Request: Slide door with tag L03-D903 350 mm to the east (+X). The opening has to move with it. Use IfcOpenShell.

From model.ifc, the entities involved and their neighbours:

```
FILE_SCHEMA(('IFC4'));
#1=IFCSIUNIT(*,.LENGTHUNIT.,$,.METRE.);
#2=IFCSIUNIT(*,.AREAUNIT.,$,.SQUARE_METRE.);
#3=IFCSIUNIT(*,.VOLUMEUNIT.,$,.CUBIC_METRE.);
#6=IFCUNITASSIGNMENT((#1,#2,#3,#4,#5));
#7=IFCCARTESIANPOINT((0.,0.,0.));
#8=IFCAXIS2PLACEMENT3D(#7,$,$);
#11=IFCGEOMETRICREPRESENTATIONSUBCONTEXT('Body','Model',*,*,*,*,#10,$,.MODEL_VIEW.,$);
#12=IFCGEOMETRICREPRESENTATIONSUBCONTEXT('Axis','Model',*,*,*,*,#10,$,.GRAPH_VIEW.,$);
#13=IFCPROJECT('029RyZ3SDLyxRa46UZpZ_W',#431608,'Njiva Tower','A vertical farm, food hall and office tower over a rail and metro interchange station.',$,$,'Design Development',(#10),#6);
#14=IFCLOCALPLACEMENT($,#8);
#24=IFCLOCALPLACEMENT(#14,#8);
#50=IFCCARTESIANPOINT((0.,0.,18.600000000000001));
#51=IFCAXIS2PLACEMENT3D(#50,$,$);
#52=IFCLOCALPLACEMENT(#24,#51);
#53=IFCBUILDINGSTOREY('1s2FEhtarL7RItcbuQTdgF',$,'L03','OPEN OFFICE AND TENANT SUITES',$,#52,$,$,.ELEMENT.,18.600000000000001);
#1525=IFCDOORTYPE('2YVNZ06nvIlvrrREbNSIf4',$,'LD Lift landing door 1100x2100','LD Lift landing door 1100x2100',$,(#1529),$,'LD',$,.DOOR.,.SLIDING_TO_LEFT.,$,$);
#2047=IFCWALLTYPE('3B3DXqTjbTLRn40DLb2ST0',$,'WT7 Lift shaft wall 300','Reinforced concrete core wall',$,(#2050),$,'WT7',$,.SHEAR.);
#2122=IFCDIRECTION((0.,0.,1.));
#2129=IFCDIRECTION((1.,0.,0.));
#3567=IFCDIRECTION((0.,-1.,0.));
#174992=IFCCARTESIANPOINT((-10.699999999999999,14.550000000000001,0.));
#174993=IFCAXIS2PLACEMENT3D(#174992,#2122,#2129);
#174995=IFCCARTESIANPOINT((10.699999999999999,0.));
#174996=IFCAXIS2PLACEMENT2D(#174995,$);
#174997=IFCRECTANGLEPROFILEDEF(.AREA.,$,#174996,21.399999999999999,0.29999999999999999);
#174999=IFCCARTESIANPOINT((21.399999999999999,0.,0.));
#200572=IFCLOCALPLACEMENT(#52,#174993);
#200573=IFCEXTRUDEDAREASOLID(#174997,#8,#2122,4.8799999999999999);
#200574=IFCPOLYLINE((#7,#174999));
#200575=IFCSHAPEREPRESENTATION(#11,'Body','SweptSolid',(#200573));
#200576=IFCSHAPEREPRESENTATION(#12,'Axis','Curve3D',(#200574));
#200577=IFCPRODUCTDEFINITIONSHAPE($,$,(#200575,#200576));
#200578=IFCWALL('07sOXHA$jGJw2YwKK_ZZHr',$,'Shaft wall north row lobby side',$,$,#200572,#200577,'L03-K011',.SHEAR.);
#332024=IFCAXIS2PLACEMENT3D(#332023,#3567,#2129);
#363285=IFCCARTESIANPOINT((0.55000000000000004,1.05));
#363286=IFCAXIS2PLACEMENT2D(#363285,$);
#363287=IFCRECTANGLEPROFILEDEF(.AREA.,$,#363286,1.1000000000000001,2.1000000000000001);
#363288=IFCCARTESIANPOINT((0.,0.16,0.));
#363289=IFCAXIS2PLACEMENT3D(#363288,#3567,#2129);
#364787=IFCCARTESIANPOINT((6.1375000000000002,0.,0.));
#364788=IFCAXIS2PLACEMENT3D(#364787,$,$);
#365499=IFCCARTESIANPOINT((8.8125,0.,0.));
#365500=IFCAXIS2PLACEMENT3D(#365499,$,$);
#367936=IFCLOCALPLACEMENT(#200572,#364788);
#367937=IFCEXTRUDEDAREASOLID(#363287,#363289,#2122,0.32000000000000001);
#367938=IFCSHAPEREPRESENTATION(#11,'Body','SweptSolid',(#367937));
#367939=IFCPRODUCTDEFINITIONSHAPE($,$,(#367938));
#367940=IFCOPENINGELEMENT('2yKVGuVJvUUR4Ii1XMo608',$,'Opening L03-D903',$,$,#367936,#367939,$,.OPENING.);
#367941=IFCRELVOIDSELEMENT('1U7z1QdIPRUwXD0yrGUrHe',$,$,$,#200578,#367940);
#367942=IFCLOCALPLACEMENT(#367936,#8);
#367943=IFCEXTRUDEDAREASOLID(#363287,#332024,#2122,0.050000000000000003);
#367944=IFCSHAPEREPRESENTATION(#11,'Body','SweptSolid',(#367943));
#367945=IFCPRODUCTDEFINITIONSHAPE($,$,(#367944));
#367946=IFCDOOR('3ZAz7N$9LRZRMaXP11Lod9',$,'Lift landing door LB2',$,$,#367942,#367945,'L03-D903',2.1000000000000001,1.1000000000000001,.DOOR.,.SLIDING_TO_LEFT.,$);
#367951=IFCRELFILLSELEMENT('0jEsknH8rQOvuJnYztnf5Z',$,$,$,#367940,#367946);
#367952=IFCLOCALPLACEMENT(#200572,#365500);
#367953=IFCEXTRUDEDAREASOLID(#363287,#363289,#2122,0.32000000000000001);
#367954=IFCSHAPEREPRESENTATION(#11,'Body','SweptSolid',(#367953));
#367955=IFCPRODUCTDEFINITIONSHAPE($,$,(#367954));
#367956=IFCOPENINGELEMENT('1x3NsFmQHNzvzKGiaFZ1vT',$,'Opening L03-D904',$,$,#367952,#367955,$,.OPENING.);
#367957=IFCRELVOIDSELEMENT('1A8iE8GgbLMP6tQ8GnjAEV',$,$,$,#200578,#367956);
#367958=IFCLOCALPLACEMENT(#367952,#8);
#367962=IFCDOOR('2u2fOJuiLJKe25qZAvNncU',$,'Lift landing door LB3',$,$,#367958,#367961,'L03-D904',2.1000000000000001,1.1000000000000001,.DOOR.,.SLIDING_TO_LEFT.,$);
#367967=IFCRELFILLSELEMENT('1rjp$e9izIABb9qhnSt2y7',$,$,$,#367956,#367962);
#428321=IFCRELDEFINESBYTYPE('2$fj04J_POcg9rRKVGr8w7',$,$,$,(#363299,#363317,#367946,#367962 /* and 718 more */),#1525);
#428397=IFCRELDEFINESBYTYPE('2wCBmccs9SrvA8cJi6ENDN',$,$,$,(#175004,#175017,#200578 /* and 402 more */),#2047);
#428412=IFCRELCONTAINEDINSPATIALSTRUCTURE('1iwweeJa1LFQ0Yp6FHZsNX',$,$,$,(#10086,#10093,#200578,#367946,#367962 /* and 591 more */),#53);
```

```python
import ifcopenshell
import ifcopenshell.api.geometry
import ifcopenshell.util.placement

model = ifcopenshell.open("model.ifc")

door = model.by_guid("3ZAz7N$9LRZRMaXP11Lod9")
opening = door.FillsVoids[0].RelatingOpeningElement
wall = opening.VoidsElements[0].RelatingBuildingElement

wall_matrix = ifcopenshell.util.placement.get_local_placement(wall.ObjectPlacement)
shift = wall_matrix[:3, 0] * 0.35
before = ifcopenshell.util.placement.get_local_placement(door.ObjectPlacement)[:3, 3].copy()

# The door is placed relative to its opening, so it follows when the opening moves.
matrix = ifcopenshell.util.placement.get_local_placement(opening.ObjectPlacement)
matrix[:3, 3] += shift
ifcopenshell.api.geometry.edit_object_placement(
    model, product=opening, matrix=matrix, is_si=False, should_transform_children=True
)

after = ifcopenshell.util.placement.get_local_placement(door.ObjectPlacement)[:3, 3]
print("door moved by", (after - before).round(3) + 0.0)

model.write("model_rev.ifc")
```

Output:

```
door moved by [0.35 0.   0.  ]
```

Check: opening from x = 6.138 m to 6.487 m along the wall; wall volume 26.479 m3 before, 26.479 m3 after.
